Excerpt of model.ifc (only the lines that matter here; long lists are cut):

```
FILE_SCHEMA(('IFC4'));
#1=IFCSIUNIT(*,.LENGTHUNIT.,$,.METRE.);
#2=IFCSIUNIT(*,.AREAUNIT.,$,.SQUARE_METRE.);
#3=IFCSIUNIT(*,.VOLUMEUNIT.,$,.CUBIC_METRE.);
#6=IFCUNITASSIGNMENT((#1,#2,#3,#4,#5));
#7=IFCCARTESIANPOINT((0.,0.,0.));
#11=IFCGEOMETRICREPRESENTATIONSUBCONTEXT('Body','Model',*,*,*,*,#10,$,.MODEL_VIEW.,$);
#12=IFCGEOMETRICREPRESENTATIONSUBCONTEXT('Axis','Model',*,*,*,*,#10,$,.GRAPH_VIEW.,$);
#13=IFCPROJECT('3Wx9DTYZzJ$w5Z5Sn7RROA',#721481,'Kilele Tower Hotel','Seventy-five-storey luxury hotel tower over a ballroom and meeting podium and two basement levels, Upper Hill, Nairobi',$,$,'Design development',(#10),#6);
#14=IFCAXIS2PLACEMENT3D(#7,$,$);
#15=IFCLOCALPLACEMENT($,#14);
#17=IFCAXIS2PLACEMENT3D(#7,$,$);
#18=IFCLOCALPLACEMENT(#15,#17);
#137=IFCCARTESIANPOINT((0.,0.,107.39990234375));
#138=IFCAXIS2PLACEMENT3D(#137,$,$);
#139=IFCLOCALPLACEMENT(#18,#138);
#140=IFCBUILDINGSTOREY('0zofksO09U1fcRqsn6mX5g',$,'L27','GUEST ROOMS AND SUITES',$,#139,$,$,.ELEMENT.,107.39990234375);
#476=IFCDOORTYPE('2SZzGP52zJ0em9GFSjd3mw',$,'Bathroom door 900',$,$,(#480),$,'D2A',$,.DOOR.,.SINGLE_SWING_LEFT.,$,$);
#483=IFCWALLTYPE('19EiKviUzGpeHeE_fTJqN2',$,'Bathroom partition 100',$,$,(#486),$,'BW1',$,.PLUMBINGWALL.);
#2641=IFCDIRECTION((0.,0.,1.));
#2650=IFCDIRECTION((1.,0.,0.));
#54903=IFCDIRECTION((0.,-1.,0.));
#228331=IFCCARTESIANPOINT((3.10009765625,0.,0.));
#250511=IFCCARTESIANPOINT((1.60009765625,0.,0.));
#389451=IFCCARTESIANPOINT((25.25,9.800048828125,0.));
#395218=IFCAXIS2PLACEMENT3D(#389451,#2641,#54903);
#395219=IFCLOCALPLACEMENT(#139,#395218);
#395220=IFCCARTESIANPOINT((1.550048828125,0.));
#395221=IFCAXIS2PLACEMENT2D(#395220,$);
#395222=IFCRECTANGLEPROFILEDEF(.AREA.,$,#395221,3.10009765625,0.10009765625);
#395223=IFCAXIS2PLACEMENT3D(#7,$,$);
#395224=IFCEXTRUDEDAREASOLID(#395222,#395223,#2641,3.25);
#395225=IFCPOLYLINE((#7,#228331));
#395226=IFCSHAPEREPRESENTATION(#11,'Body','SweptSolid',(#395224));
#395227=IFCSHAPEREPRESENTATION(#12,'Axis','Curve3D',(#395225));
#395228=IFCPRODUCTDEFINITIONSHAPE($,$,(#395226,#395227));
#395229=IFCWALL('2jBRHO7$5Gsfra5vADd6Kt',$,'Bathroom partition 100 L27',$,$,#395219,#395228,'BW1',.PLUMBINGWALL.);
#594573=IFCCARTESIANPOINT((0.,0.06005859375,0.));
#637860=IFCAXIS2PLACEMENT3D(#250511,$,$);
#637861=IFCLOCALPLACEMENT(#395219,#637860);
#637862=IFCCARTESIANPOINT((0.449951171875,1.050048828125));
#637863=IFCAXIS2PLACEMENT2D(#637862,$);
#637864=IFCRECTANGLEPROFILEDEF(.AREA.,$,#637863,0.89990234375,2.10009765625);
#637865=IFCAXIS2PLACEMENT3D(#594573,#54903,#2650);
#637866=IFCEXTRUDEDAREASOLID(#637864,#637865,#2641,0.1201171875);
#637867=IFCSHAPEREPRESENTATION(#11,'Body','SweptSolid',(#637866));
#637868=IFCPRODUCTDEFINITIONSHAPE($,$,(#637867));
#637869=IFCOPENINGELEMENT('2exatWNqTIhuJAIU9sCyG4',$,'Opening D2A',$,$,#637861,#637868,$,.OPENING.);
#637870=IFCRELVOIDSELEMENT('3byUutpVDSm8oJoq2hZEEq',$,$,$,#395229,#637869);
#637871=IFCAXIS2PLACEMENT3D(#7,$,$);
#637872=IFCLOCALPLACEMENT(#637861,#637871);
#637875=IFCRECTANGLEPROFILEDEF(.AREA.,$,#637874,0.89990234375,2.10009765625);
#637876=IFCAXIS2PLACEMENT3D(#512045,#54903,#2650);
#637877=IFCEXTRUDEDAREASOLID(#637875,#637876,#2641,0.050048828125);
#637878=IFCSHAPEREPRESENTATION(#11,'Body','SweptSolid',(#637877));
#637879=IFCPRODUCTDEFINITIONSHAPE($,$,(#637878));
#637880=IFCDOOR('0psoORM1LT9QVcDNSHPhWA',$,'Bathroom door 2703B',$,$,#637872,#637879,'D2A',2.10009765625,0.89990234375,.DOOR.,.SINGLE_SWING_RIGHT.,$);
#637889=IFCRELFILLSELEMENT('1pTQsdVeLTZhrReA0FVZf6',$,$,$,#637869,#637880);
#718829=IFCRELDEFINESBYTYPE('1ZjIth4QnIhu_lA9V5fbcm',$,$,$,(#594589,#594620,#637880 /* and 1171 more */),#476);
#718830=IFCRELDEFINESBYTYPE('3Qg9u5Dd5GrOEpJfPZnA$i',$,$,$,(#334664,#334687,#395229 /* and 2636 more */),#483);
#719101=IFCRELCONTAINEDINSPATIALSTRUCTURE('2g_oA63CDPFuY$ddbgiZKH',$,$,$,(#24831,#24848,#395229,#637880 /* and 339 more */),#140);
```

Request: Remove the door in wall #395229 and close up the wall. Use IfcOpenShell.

```python
import ifcopenshell
import ifcopenshell.api.feature
import ifcopenshell.api.root
import ifcopenshell.geom
import ifcopenshell.util.shape

model = ifcopenshell.open("model.ifc")
settings = ifcopenshell.geom.settings()


def volume(element):
    """Net volume in cubic metres, openings subtracted."""
    shape = ifcopenshell.geom.create_shape(settings, element)
    return ifcopenshell.util.shape.get_volume(shape.geometry)


door = model.by_id(637880)
opening = door.FillsVoids[0].RelatingOpeningElement
wall = opening.VoidsElements[0].RelatingBuildingElement
before = volume(wall)

ifcopenshell.api.root.remove_product(model, product=door)
ifcopenshell.api.feature.remove_feature(model, feature=opening)

after = volume(wall)

print(f"wall volume {before:.3f} -> {after:.3f} m3")

model.write("model_v2.ifc")
```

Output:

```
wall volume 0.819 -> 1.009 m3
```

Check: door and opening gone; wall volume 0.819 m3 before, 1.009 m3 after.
